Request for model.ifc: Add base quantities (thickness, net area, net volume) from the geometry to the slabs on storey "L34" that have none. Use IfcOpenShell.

First a look at what the model holds.

```python
import ifcopenshell
import ifcopenshell.util.element
import ifcopenshell.util.unit

model = ifcopenshell.open("model.ifc")
print(model.schema)
for unit_type in ("LENGTHUNIT", "AREAUNIT", "VOLUMEUNIT"):
    print(unit_type, ifcopenshell.util.unit.calculate_unit_scale(model, unit_type))
storey = next(s for s in model.by_type("IfcBuildingStorey") if s.Name == "L34")
slabs = [e for e in ifcopenshell.util.element.get_decomposition(storey) if e.is_a("IfcSlab")]
for e in sorted(slabs, key=lambda e: e.id()):
    print(e.id(), e.is_a(), e.Name, list(ifcopenshell.util.element.get_psets(e, qtos_only=True)), sep=" | ")
```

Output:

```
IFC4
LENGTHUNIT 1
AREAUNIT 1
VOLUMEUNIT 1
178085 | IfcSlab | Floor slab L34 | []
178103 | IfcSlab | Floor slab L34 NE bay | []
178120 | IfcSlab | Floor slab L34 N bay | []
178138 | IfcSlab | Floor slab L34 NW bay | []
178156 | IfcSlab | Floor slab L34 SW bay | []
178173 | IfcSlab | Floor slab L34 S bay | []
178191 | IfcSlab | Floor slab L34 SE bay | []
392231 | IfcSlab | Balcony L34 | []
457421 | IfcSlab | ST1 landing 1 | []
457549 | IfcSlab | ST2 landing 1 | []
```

```python
import ifcopenshell
import ifcopenshell.api.pset
import ifcopenshell.geom
import ifcopenshell.util.element
import ifcopenshell.util.shape
import ifcopenshell.util.unit

model = ifcopenshell.open("model.ifc")
unit_scale = ifcopenshell.util.unit.calculate_unit_scale(model)
area_scale = ifcopenshell.util.unit.calculate_unit_scale(model, "AREAUNIT")
volume_scale = ifcopenshell.util.unit.calculate_unit_scale(model, "VOLUMEUNIT")
settings = ifcopenshell.geom.settings()

storey = next(s for s in model.by_type("IfcBuildingStorey") if s.Name == "L34")
slabs = [e for e in ifcopenshell.util.element.get_decomposition(storey) if e.is_a("IfcSlab")]

for e in sorted(slabs, key=lambda e: e.id()):
    if ifcopenshell.util.element.get_psets(e, qtos_only=True, should_inherit=False):
        continue
    # Geometry comes back in metres, in the element's own axes.
    shape = ifcopenshell.geom.create_shape(settings, e)
    values = {
        "Width": ifcopenshell.util.shape.get_z(shape.geometry) / unit_scale,
        "NetArea": ifcopenshell.util.shape.get_footprint_area(shape.geometry) / area_scale,
        "NetVolume": ifcopenshell.util.shape.get_volume(shape.geometry) / volume_scale,
    }
    qto = ifcopenshell.api.pset.add_qto(model, product=e, name="Qto_SlabBaseQuantities")
    ifcopenshell.api.pset.edit_qto(model, qto=qto, properties=values)
    print(e.id(), {k: round(v, 3) for k, v in values.items()})

model.write("model_v2.ifc")
```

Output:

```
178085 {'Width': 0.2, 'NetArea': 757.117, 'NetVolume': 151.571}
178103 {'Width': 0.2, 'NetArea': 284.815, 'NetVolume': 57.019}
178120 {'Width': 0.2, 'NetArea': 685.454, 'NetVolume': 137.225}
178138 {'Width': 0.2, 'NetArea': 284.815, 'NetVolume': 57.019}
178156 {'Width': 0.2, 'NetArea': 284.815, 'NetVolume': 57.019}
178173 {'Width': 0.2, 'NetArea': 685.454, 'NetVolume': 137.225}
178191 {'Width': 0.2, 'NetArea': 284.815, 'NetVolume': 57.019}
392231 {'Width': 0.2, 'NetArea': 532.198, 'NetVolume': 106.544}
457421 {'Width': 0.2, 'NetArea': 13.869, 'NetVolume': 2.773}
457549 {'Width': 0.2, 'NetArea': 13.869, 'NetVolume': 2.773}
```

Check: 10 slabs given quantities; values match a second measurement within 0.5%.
